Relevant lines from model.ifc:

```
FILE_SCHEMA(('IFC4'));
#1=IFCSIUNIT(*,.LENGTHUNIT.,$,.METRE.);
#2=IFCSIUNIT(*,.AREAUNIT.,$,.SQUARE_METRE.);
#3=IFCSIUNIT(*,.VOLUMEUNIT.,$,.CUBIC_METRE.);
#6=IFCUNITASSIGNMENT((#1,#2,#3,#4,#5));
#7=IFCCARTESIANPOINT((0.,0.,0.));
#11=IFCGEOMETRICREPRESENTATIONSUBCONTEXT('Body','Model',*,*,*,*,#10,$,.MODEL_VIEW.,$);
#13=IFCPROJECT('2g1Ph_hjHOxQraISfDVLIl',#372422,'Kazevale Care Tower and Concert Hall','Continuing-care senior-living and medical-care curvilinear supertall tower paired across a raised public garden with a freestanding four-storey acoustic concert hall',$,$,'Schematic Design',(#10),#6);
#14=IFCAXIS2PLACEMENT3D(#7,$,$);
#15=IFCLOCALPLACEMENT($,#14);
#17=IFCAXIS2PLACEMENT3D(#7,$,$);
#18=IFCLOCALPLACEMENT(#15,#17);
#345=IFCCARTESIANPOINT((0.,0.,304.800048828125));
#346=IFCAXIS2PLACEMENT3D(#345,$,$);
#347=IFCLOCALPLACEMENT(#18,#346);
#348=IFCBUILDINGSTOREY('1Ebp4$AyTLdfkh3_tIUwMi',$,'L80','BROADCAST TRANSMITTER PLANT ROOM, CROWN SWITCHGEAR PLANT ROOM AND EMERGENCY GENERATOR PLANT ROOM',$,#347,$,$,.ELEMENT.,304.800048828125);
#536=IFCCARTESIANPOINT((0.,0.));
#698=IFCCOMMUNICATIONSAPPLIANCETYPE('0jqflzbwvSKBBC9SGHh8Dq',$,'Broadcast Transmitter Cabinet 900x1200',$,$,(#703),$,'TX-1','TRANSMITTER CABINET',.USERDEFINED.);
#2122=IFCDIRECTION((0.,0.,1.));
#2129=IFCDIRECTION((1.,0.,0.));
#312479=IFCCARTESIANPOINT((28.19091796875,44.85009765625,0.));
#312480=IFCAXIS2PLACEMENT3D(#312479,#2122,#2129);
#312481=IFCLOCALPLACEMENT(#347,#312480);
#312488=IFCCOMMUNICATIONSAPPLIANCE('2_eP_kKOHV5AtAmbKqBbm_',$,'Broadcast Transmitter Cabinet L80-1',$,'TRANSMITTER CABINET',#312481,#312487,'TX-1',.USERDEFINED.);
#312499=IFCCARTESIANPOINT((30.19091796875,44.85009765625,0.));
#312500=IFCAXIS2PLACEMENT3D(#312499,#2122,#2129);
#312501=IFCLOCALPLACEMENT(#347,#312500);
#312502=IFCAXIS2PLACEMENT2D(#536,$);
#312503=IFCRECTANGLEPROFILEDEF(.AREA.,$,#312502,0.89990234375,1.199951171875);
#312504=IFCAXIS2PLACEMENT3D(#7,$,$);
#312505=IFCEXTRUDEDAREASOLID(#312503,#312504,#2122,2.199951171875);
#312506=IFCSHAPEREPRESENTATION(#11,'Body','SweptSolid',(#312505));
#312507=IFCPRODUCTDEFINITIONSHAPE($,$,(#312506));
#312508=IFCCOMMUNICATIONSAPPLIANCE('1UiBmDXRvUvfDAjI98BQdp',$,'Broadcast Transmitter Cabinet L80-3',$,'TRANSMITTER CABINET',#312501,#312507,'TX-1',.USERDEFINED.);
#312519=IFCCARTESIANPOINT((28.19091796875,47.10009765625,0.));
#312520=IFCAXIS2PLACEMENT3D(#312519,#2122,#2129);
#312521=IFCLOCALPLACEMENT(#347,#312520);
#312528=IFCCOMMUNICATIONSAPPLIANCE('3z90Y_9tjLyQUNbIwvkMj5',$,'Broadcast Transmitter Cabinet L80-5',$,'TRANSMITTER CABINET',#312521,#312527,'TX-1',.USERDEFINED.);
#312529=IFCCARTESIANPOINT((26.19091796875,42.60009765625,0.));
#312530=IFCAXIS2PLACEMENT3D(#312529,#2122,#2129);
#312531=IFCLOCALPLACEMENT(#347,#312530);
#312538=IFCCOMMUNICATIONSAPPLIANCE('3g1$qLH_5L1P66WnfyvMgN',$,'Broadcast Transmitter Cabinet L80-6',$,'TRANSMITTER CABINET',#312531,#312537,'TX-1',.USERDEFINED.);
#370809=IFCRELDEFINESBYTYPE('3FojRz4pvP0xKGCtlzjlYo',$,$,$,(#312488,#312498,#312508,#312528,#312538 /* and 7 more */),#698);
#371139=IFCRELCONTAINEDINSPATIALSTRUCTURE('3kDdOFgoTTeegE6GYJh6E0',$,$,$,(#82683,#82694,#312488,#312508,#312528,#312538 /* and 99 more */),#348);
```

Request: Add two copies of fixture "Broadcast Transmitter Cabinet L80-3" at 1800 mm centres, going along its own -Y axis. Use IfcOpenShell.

```python
import ifcopenshell
import ifcopenshell.api.geometry
import ifcopenshell.api.root
import ifcopenshell.util.element
import ifcopenshell.util.placement
import ifcopenshell.util.unit

model = ifcopenshell.open("model.ifc")
unit_scale = ifcopenshell.util.unit.calculate_unit_scale(model)

source = model.by_guid("1UiBmDXRvUvfDAjI98BQdp")
base = ifcopenshell.util.placement.get_local_placement(source.ObjectPlacement)
step = -base[:3, 1] * 1.8 / unit_scale

for i in range(1, 3):
    copy = ifcopenshell.api.root.copy_class(model, product=source)
    copy.Representation = ifcopenshell.util.element.copy_deep(
        model, source.Representation, exclude=["IfcGeometricRepresentationContext", "IfcRepresentationMap"]
    )
    copy.Tag = None
    matrix = base.copy()
    matrix[:3, 3] += i * step
    print("added at", matrix[:3, 3].round(3) + 0.0)
    ifcopenshell.api.geometry.edit_object_placement(model, product=copy, matrix=matrix, is_si=False)

model.write("model_rev.ifc")
```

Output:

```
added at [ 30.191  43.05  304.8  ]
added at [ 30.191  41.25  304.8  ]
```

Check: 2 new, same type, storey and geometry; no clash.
